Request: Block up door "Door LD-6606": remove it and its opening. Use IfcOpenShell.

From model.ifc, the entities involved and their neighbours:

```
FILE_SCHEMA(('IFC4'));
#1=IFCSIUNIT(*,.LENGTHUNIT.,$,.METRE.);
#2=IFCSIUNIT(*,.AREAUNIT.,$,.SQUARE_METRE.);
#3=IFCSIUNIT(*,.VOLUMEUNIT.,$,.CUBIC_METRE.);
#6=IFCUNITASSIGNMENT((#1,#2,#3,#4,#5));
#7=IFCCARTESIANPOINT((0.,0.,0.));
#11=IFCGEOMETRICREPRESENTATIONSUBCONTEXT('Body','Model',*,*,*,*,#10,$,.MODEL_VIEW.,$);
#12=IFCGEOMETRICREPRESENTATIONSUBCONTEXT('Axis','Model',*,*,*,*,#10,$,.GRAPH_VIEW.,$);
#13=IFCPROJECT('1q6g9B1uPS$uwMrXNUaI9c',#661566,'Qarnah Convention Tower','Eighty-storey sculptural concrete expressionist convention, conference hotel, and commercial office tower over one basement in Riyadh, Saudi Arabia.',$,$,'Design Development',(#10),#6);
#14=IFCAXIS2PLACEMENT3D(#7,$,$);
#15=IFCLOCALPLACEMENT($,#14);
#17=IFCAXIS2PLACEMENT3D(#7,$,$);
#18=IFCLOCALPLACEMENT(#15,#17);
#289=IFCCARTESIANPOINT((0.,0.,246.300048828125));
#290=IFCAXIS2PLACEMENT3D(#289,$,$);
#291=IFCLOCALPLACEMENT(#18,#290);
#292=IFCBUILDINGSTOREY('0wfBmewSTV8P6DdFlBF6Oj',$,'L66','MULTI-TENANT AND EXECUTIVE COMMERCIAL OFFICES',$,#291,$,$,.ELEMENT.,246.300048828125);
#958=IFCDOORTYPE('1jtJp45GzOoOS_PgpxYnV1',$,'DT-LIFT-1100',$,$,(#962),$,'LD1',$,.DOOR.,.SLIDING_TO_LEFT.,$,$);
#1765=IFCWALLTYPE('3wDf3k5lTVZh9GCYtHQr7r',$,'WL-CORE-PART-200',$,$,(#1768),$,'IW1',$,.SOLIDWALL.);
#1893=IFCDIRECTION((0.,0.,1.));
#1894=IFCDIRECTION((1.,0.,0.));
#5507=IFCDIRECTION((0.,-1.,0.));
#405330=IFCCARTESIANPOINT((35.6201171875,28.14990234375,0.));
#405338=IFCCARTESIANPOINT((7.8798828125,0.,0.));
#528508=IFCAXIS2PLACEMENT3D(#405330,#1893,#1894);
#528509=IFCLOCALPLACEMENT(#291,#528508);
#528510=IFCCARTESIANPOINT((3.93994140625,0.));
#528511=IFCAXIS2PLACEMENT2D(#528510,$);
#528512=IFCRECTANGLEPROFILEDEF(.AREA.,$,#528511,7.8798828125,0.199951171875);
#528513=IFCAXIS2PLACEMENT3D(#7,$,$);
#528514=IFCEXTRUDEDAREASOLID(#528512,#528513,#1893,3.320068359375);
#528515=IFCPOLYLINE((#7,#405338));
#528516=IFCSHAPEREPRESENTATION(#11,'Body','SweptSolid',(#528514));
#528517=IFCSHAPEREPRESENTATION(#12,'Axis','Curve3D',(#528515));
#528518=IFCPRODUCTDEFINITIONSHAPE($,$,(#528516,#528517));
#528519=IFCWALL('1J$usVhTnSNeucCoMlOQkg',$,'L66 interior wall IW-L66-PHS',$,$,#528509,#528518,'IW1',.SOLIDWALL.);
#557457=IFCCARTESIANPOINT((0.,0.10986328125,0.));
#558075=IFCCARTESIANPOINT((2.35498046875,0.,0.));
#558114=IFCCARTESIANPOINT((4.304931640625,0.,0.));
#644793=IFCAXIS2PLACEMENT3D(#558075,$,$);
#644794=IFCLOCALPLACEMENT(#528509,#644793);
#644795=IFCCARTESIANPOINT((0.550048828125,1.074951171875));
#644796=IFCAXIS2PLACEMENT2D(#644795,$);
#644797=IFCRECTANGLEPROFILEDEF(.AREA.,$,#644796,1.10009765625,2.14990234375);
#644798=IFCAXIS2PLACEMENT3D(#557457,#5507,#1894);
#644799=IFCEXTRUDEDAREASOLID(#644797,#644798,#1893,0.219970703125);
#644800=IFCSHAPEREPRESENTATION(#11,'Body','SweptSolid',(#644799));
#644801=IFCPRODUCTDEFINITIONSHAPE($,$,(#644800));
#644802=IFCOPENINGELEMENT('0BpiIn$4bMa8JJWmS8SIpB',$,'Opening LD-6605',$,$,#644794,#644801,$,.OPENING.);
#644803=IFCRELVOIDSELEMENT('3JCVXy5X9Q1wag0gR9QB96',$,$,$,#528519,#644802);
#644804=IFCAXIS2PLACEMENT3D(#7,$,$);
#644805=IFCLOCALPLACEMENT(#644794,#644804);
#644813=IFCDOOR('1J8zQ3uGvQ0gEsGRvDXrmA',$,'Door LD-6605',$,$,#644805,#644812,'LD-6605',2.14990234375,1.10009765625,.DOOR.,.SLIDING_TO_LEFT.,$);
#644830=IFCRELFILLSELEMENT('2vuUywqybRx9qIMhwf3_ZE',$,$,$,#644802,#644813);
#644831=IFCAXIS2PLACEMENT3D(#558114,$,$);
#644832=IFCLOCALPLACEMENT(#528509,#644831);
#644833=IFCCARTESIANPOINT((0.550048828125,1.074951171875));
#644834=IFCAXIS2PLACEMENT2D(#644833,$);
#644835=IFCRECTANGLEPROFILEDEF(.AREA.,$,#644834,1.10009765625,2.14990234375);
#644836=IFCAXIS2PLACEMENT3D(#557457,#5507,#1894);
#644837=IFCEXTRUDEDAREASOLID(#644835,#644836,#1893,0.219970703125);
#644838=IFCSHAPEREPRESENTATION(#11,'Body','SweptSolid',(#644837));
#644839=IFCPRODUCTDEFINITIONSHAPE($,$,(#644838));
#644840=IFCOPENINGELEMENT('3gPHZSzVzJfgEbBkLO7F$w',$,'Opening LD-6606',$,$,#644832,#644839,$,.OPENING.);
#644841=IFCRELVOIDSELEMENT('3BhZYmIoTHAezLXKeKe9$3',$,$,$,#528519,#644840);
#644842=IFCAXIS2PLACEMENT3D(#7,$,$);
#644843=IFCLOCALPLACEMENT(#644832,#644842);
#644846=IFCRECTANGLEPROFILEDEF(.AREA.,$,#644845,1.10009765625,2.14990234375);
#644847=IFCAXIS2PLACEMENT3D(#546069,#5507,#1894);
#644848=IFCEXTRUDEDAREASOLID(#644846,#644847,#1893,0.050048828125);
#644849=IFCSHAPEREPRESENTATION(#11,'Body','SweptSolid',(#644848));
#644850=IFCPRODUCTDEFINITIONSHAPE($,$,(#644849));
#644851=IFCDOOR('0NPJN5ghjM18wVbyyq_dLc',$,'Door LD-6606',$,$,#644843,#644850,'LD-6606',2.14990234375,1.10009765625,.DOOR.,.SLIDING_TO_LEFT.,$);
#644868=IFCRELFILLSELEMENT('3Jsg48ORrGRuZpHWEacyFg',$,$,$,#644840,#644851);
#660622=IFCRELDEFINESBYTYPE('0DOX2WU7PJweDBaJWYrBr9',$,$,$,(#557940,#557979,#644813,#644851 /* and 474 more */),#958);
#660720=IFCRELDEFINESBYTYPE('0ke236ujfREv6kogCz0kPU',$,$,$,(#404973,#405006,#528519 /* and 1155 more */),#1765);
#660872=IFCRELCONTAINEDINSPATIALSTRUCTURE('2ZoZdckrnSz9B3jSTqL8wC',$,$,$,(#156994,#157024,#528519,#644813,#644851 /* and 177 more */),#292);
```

```python
import ifcopenshell
import ifcopenshell.api.feature
import ifcopenshell.api.root
import ifcopenshell.geom
import ifcopenshell.util.shape

model = ifcopenshell.open("model.ifc")
settings = ifcopenshell.geom.settings()


def volume(element):
    """Net volume in cubic metres, openings subtracted."""
    shape = ifcopenshell.geom.create_shape(settings, element)
    return ifcopenshell.util.shape.get_volume(shape.geometry)


door = model.by_guid("0NPJN5ghjM18wVbyyq_dLc")
opening = door.FillsVoids[0].RelatingOpeningElement
wall = opening.VoidsElements[0].RelatingBuildingElement
before = volume(wall)

ifcopenshell.api.root.remove_product(model, product=door)
ifcopenshell.api.feature.remove_feature(model, feature=opening)

after = volume(wall)

print(f"wall volume {before:.3f} -> {after:.3f} m3")

model.write("model-out.ifc")
```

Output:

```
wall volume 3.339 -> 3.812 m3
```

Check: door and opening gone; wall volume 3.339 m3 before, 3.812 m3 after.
